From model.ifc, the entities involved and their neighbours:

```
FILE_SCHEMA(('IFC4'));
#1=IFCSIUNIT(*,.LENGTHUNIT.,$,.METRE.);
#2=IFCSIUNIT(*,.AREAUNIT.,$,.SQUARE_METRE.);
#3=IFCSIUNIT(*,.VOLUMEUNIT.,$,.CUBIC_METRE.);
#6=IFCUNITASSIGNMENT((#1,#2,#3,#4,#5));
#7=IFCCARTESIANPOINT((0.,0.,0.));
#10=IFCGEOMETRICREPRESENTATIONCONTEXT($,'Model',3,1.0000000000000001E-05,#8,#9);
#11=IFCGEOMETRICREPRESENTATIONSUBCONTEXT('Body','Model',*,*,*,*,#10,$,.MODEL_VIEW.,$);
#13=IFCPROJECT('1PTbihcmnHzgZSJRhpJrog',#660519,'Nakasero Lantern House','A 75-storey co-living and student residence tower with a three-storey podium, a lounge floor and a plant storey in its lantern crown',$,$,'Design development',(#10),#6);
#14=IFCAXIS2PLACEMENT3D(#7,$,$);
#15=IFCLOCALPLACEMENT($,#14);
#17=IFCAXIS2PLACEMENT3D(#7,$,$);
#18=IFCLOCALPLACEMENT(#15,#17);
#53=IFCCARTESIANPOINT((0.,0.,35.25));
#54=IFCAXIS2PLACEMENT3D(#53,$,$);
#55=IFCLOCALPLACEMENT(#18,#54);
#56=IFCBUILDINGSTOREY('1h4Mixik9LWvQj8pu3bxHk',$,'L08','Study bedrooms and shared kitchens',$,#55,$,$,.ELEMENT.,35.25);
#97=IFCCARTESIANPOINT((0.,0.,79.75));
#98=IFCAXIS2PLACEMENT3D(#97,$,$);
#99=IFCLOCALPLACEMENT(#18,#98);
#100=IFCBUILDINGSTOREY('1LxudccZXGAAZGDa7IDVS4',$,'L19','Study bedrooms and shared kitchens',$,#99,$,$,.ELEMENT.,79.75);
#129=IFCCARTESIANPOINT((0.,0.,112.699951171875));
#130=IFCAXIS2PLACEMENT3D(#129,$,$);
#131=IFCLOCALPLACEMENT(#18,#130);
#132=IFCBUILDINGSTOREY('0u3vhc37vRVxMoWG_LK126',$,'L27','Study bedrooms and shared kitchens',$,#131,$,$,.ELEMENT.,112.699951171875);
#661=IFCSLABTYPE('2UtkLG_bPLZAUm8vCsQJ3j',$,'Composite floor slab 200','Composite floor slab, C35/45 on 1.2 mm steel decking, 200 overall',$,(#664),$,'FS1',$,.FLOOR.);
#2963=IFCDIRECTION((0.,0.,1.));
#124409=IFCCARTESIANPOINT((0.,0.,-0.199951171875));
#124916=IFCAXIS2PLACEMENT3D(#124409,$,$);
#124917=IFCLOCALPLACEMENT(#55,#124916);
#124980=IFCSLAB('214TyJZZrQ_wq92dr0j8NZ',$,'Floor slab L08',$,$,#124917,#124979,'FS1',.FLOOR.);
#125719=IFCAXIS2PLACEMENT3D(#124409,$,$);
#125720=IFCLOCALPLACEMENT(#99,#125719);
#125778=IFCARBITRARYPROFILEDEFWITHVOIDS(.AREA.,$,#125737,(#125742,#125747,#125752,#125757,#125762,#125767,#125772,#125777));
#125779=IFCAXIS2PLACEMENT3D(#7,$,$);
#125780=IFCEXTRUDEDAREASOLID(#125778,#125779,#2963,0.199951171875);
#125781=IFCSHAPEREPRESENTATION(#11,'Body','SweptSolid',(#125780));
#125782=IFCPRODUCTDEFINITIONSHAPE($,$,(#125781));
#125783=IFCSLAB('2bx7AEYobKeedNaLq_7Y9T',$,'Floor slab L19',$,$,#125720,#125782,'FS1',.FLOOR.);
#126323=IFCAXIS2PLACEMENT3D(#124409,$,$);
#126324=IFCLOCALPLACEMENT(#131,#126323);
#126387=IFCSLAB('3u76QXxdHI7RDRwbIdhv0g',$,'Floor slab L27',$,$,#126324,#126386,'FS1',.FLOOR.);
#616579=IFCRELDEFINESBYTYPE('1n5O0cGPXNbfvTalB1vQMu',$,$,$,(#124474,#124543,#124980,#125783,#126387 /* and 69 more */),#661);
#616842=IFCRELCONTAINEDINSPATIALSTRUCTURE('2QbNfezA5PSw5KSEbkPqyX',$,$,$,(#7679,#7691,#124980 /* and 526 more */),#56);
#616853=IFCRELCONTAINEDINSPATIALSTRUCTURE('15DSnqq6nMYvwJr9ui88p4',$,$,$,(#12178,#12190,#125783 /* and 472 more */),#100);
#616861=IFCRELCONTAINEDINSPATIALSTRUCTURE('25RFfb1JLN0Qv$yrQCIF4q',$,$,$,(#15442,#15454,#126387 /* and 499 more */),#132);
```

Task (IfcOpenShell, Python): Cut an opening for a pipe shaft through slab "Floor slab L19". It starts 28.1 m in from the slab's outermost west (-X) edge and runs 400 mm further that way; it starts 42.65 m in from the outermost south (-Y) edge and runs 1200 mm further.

```python
import numpy as np
import ifcopenshell
import ifcopenshell.api.feature
import ifcopenshell.api.geometry
import ifcopenshell.api.root
import ifcopenshell.geom
import ifcopenshell.util.placement
import ifcopenshell.util.representation
import ifcopenshell.util.shape
import ifcopenshell.util.unit

model = ifcopenshell.open("model.ifc")
unit_scale = ifcopenshell.util.unit.calculate_unit_scale(model)
settings = ifcopenshell.geom.settings()


def volume(element):
    """Net volume in cubic metres, openings subtracted."""
    shape = ifcopenshell.geom.create_shape(settings, element)
    return ifcopenshell.util.shape.get_volume(shape.geometry)


slab = model.by_id(125783)
before = volume(slab)

# Extent in the slab's own axes, in metres. The edges named are its -X and -Y sides.
slab_shape = ifcopenshell.geom.create_shape(settings, slab)
vertices = ifcopenshell.util.shape.get_vertices(slab_shape.geometry)
x_min, y_min, bottom = vertices.min(axis=0)
top = vertices[:, 2].max()

opening = ifcopenshell.api.root.create_entity(model, ifc_class="IfcOpeningElement", name="Pipe shaft opening", predefined_type="OPENING")
context = ifcopenshell.util.representation.get_context(model, "Model", "Body", "MODEL_VIEW")
width, depth = 0.4, 1.2
outline = [(0.0, 0.0), (width, 0.0), (width, depth), (0.0, depth), (0.0, 0.0)]
# Overshoot both faces by 50 mm so the cut is clean.
shape = ifcopenshell.api.geometry.add_slab_representation(
    model, context=context, depth=top - bottom + 0.1, polyline=outline
)
ifcopenshell.api.geometry.assign_representation(model, product=opening, representation=shape)

matrix = ifcopenshell.util.placement.get_local_placement(slab.ObjectPlacement)
matrix[:, 3] = matrix @ np.append(np.array([x_min + 28.1, y_min + 42.65, bottom - 0.05]) / unit_scale, 1.0)
ifcopenshell.api.geometry.edit_object_placement(model, product=opening, matrix=matrix, is_si=False)
ifcopenshell.api.feature.add_feature(model, feature=opening, element=slab)

after = volume(slab)

print(f"slab volume {before:.3f} -> {after:.3f} m3")

model.write("model_v2.ifc")
```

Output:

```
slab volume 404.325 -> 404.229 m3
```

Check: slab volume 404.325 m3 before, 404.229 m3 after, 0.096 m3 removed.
